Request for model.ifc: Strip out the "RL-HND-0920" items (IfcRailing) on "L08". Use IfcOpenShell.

First a look at what the model holds.

```python
import ifcopenshell
import ifcopenshell.util.element

model = ifcopenshell.open("model.ifc")
print(model.schema)
storey = next(s for s in model.by_type("IfcBuildingStorey") if s.Name == "L08")
railings = [e for e in ifcopenshell.util.element.get_decomposition(storey) if e.is_a("IfcRailing")]
seen = {}
for e in railings:
    element_type = ifcopenshell.util.element.get_type(e)
    name = element_type.Name if element_type not in (None, e) else None
    seen[name] = seen.get(name, 0) + 1
for name, count in sorted(seen.items(), key=str):
    print(count, "x", name)
```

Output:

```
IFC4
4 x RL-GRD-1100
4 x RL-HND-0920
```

```python
import ifcopenshell
import ifcopenshell.api.root
import ifcopenshell.util.element

model = ifcopenshell.open("model.ifc")

storey = next(s for s in model.by_type("IfcBuildingStorey") if s.Name == "L08")
railings = [e for e in ifcopenshell.util.element.get_decomposition(storey) if e.is_a("IfcRailing")]
targets = [e for e in railings if (t := ifcopenshell.util.element.get_type(e)) not in (None, e) and t.Name == "RL-HND-0920"]

for e in targets:
    ifcopenshell.api.root.remove_product(model, product=e)
print(len(targets), "removed")

model.write("model_updated.ifc")
```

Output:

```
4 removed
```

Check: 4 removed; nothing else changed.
